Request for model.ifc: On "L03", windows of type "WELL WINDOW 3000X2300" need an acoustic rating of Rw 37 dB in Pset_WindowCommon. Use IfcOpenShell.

First a look at what the model holds.

```python
import ifcopenshell
import ifcopenshell.util.element

model = ifcopenshell.open("model.ifc")
print(model.schema)
storey = next(s for s in model.by_type("IfcBuildingStorey") if s.Name == "L03")
windows = [e for e in ifcopenshell.util.element.get_decomposition(storey) if e.is_a("IfcWindow")]
seen = {}
for e in windows:
    element_type = ifcopenshell.util.element.get_type(e)
    key = (element_type.Name if element_type != e and element_type else None, ifcopenshell.util.element.get_pset(e, "Pset_WindowCommon", "AcousticRating"))
    seen[key] = seen.get(key, 0) + 1
for (name, value), count in sorted(seen.items(), key=str):
    print(count, "x", name, "|", value)
```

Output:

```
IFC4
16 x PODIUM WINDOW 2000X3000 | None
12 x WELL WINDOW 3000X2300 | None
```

```python
import ifcopenshell
import ifcopenshell.api.pset
import ifcopenshell.util.element

model = ifcopenshell.open("model.ifc")

storey = next(s for s in model.by_type("IfcBuildingStorey") if s.Name == "L03")
windows = [e for e in ifcopenshell.util.element.get_decomposition(storey) if e.is_a("IfcWindow")]

count = 0
for e in windows:
    element_type = ifcopenshell.util.element.get_type(e)
    if element_type in (None, e) or element_type.Name != "WELL WINDOW 3000X2300":
        continue
    found = ifcopenshell.util.element.get_pset(e, "Pset_WindowCommon", should_inherit=False)
    if found:
        pset = model.by_id(found["id"])
        if len(ifcopenshell.util.element.get_elements_by_pset(pset)) > 1:
            pset = ifcopenshell.api.pset.unshare_pset(model, products=[e], pset=pset)[0]
    else:
        pset = ifcopenshell.api.pset.add_pset(model, product=e, name="Pset_WindowCommon")
    ifcopenshell.api.pset.edit_pset(model, pset=pset, properties={"AcousticRating": "Rw 37 dB"})
    count += 1

print(count, "windows updated")

model.write("model-out.ifc")
```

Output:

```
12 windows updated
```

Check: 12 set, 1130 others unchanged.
